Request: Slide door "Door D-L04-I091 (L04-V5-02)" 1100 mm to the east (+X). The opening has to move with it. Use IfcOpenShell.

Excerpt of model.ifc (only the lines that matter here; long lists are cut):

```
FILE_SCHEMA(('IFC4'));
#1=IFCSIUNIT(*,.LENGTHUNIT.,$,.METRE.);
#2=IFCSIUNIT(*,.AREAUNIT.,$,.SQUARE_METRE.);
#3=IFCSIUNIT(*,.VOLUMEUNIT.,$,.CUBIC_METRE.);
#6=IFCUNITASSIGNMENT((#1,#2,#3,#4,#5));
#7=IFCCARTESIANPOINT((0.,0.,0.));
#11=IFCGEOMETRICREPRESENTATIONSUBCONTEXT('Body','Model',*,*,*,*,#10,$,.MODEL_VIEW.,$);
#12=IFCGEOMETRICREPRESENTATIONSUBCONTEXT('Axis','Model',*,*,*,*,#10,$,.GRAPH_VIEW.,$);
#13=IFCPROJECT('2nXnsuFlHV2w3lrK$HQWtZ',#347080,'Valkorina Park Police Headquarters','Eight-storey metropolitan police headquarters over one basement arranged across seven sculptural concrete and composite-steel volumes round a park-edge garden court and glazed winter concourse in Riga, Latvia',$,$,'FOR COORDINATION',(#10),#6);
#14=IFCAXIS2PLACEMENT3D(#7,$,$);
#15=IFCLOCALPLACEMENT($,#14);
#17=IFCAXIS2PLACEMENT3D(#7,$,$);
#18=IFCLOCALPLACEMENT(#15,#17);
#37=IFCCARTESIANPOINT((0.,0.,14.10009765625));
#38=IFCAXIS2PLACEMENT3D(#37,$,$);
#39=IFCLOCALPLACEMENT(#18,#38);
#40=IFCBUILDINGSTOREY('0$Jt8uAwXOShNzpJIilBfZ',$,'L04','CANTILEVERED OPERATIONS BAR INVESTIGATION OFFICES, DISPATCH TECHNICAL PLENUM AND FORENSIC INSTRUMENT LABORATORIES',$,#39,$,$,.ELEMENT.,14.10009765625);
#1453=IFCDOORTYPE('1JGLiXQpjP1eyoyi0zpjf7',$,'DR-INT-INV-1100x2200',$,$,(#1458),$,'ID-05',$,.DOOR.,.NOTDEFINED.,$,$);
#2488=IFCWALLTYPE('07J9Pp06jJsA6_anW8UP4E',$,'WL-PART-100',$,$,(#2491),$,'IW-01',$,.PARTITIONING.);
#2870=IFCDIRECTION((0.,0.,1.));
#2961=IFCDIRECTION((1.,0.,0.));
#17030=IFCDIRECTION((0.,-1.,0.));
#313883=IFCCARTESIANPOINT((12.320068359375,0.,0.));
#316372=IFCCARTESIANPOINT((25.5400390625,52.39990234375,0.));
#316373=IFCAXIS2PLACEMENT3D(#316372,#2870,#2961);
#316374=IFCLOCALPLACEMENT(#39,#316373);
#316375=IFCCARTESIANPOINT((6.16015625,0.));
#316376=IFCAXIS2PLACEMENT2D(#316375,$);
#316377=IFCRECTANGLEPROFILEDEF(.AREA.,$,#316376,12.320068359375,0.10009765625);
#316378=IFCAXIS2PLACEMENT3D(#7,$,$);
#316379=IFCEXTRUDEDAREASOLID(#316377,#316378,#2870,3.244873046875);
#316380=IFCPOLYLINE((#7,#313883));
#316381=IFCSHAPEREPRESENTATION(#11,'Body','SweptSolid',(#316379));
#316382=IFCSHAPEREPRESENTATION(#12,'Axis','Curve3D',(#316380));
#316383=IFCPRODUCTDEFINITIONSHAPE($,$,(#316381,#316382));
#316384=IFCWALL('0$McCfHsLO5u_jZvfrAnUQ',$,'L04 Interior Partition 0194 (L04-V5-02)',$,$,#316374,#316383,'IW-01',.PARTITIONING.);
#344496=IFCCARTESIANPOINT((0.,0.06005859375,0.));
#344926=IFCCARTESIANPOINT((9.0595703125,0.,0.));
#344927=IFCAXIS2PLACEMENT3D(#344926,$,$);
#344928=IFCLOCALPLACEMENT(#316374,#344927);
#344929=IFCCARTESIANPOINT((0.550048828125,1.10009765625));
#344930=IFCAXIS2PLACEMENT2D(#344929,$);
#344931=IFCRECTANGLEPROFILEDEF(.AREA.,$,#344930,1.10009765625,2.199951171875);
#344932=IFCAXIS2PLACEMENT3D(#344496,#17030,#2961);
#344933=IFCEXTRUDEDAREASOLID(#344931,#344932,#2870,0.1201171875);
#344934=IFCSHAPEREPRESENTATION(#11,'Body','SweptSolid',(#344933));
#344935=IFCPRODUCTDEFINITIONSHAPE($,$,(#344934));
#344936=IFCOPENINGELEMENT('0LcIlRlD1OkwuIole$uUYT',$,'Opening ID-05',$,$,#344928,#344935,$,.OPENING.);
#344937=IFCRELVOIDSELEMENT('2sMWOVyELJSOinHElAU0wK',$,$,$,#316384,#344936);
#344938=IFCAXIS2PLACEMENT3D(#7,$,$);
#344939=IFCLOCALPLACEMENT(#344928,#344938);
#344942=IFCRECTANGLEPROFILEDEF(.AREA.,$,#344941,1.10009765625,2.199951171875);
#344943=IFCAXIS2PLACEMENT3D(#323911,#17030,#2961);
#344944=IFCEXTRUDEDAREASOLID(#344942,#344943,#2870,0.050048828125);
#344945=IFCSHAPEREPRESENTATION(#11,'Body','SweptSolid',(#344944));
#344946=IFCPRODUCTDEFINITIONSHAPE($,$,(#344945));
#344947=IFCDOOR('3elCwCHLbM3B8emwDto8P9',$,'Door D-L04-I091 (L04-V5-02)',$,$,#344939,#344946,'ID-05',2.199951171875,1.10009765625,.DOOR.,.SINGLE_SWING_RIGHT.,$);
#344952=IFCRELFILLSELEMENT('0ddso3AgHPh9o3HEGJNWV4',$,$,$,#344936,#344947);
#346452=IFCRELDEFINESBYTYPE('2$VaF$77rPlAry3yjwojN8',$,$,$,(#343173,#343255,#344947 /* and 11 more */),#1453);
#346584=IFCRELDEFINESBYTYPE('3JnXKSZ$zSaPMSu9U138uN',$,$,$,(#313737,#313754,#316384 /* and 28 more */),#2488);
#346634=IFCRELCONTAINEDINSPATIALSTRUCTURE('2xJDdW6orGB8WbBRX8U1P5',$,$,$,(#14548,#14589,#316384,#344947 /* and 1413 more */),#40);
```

```python
import ifcopenshell
import ifcopenshell.api.geometry
import ifcopenshell.util.placement
import ifcopenshell.util.unit

model = ifcopenshell.open("model.ifc")
unit_scale = ifcopenshell.util.unit.calculate_unit_scale(model)

door = model.by_guid("3elCwCHLbM3B8emwDto8P9")
opening = door.FillsVoids[0].RelatingOpeningElement
wall = opening.VoidsElements[0].RelatingBuildingElement

wall_matrix = ifcopenshell.util.placement.get_local_placement(wall.ObjectPlacement)
shift = wall_matrix[:3, 0] * 1.1 / unit_scale
before = ifcopenshell.util.placement.get_local_placement(door.ObjectPlacement)[:3, 3].copy()

# The door is placed relative to its opening, so it follows when the opening moves.
matrix = ifcopenshell.util.placement.get_local_placement(opening.ObjectPlacement)
matrix[:3, 3] += shift
ifcopenshell.api.geometry.edit_object_placement(
    model, product=opening, matrix=matrix, is_si=False, should_transform_children=True
)

after = ifcopenshell.util.placement.get_local_placement(door.ObjectPlacement)[:3, 3]
print("door moved by", (after - before).round(3) + 0.0)

model.write("model_rev.ifc")
```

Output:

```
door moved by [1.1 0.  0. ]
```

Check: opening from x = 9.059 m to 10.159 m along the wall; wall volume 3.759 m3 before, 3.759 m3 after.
